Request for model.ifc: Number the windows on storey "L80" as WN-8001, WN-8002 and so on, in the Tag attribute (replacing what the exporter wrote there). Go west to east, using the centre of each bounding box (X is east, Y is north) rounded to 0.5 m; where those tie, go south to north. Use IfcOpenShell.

First a look at what the model holds.

```python
import ifcopenshell
import ifcopenshell.util.element
import ifcopenshell.util.placement

model = ifcopenshell.open("model.ifc")
print(model.schema)
storey = next(s for s in model.by_type("IfcBuildingStorey") if s.Name == "L80")
windows = [e for e in ifcopenshell.util.element.get_decomposition(storey) if e.is_a("IfcWindow")]
for e in sorted(windows, key=lambda e: e.id()):
    origin = ifcopenshell.util.placement.get_local_placement(e.ObjectPlacement)[:3, 3]
    print(e.id(), e.Tag, e.Name, origin.round(2) + 0.0, sep=" | ")
```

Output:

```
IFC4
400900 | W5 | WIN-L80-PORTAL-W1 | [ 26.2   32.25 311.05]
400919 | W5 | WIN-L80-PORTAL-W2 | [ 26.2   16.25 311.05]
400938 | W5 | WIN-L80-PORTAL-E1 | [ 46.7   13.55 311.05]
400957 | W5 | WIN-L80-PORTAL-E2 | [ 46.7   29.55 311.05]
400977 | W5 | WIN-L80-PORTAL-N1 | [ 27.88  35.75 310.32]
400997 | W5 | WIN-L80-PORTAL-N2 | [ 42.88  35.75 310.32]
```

```python
import ifcopenshell
import ifcopenshell.geom
import ifcopenshell.util.element
import ifcopenshell.util.shape

model = ifcopenshell.open("model.ifc")
settings = ifcopenshell.geom.settings()
settings.set("use-world-coords", True)


def centre(element):
    shape = ifcopenshell.geom.create_shape(settings, element)
    return ifcopenshell.util.shape.get_bbox_centroid(shape.geometry)


storey = next(s for s in model.by_type("IfcBuildingStorey") if s.Name == "L80")
windows = [e for e in ifcopenshell.util.element.get_decomposition(storey) if e.is_a("IfcWindow")]

# Insertion points can sit at a corner or the storey origin, so sort by the geometry (in metres).
centres = {e: centre(e) for e in windows}
windows.sort(key=lambda e: (round(centres[e][0] / 0.5), centres[e][1]))

for i, e in enumerate(windows, start=1):
    number = f"WN-80{i:02d}"
    e.Tag = number
    print(e.id(), number)

model.write("model_edited.ifc")
```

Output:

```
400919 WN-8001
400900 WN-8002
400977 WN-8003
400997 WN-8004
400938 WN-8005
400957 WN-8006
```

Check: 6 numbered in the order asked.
